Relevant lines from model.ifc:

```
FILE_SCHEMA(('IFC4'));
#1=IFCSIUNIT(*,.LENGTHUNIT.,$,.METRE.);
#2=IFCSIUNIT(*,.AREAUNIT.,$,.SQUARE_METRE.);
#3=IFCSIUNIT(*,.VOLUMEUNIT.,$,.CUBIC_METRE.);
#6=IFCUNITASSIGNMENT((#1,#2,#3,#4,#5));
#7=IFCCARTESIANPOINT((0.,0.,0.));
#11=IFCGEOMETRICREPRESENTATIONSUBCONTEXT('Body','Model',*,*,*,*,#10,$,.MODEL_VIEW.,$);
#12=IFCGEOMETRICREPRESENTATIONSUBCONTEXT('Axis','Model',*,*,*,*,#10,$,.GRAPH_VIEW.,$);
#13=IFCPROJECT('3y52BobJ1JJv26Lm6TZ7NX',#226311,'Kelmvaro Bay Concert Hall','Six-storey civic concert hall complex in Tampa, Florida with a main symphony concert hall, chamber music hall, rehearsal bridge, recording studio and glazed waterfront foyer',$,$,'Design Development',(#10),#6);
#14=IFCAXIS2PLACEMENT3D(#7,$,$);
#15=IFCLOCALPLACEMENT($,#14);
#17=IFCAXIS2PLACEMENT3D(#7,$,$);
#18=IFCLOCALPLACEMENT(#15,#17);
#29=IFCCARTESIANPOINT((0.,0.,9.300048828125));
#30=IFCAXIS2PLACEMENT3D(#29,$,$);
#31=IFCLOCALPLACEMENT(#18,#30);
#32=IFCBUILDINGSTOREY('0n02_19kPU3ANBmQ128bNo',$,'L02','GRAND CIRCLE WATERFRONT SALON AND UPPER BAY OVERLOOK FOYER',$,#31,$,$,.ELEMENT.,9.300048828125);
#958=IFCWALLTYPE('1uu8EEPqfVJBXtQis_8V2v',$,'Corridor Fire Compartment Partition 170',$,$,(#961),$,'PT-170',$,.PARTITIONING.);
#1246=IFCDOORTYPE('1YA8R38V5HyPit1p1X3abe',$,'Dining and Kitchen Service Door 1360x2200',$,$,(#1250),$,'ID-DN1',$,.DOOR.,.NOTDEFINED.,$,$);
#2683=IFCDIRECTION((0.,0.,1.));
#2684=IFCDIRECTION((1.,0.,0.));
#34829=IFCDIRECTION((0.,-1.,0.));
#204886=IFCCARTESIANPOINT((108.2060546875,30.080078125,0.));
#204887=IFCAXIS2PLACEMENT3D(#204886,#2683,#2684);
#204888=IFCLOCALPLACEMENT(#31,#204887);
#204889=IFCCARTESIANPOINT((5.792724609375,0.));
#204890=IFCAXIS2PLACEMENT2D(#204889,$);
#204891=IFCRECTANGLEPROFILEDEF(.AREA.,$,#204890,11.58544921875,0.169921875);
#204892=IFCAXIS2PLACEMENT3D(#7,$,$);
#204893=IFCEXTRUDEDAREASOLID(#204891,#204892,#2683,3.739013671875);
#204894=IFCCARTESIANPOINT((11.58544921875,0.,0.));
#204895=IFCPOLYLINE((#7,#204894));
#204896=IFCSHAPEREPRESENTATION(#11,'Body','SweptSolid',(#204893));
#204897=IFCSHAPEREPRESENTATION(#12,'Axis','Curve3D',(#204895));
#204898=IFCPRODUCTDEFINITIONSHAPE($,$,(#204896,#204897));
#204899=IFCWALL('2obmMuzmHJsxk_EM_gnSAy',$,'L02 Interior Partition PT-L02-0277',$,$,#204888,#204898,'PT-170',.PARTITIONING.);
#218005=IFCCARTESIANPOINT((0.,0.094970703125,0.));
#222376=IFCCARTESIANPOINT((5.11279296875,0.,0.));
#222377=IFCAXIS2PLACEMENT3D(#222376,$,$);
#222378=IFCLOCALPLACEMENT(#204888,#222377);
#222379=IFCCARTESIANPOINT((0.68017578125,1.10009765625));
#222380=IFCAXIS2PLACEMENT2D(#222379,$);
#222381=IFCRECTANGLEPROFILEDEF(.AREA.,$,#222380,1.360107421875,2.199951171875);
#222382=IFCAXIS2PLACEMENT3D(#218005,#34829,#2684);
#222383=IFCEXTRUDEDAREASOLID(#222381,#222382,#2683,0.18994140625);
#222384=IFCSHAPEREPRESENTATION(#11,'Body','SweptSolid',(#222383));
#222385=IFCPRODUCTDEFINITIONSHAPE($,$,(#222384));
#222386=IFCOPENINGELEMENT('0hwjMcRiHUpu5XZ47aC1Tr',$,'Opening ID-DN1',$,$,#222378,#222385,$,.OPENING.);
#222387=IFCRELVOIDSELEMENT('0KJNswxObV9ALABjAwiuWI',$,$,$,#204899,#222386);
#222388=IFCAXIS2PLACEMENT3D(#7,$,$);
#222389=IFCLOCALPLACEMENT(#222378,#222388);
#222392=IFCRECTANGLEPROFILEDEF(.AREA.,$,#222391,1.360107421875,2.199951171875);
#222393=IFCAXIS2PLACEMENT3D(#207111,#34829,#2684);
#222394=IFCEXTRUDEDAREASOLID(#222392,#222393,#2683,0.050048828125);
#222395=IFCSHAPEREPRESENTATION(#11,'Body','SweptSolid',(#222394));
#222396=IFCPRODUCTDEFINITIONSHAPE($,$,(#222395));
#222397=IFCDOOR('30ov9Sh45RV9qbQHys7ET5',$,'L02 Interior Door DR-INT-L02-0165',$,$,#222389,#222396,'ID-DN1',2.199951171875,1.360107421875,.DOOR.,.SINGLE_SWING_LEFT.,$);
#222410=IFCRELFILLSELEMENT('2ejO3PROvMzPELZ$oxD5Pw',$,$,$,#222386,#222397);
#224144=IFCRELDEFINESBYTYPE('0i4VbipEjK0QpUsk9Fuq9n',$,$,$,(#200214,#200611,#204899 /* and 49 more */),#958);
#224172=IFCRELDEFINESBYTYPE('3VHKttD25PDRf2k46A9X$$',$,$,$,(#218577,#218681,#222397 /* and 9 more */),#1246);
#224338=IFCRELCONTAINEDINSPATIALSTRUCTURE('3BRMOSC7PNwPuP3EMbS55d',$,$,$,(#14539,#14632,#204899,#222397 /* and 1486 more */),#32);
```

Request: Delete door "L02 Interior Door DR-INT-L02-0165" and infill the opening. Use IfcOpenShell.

```python
import ifcopenshell
import ifcopenshell.api.feature
import ifcopenshell.api.root
import ifcopenshell.geom
import ifcopenshell.util.shape

model = ifcopenshell.open("model.ifc")
settings = ifcopenshell.geom.settings()


def volume(element):
    """Net volume in cubic metres, openings subtracted."""
    shape = ifcopenshell.geom.create_shape(settings, element)
    return ifcopenshell.util.shape.get_volume(shape.geometry)


door = model.by_guid("30ov9Sh45RV9qbQHys7ET5")
opening = door.FillsVoids[0].RelatingOpeningElement
wall = opening.VoidsElements[0].RelatingBuildingElement
before = volume(wall)

ifcopenshell.api.root.remove_product(model, product=door)
ifcopenshell.api.feature.remove_feature(model, feature=opening)

after = volume(wall)

print(f"wall volume {before:.3f} -> {after:.3f} m3")

model.write("model_rev.ifc")
```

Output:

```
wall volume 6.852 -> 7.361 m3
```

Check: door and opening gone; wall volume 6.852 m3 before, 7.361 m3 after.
